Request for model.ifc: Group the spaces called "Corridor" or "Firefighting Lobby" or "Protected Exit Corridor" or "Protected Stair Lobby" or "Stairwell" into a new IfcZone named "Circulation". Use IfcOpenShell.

First a look at what the model holds.

```python
import ifcopenshell

model = ifcopenshell.open("model.ifc")
print(model.schema)
seen = {}
for space in model.by_type("IfcSpace"):
    seen[space.LongName] = seen.get(space.LongName, 0) + 1
for name, count in sorted(seen.items(), key=str):
    print(count, "x", name)
print("zones:", [z.Name for z in model.by_type("IfcZone")][:20])
```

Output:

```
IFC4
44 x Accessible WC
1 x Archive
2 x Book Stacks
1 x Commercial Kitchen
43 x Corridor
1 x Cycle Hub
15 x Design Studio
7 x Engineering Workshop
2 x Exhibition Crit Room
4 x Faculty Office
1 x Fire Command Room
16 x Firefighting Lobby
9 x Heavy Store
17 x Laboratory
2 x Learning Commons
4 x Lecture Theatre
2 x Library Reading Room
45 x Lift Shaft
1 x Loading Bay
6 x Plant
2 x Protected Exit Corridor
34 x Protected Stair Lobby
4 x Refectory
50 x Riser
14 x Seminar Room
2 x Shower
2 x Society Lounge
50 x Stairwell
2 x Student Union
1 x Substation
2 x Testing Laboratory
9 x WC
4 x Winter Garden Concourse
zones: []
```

```python
import ifcopenshell
import ifcopenshell.api.group
import ifcopenshell.api.root

model = ifcopenshell.open("model.ifc")

names = {"Corridor", "Firefighting Lobby", "Protected Exit Corridor", "Protected Stair Lobby", "Stairwell"}
spaces = [s for s in model.by_type("IfcSpace") if s.LongName in names]

zone = ifcopenshell.api.root.create_entity(model, ifc_class="IfcZone", name="Circulation")
ifcopenshell.api.group.assign_group(model, products=spaces, group=zone)
print(len(spaces), "spaces in", zone.Name)

model.write("model_rev.ifc")
```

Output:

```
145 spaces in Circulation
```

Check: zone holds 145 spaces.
